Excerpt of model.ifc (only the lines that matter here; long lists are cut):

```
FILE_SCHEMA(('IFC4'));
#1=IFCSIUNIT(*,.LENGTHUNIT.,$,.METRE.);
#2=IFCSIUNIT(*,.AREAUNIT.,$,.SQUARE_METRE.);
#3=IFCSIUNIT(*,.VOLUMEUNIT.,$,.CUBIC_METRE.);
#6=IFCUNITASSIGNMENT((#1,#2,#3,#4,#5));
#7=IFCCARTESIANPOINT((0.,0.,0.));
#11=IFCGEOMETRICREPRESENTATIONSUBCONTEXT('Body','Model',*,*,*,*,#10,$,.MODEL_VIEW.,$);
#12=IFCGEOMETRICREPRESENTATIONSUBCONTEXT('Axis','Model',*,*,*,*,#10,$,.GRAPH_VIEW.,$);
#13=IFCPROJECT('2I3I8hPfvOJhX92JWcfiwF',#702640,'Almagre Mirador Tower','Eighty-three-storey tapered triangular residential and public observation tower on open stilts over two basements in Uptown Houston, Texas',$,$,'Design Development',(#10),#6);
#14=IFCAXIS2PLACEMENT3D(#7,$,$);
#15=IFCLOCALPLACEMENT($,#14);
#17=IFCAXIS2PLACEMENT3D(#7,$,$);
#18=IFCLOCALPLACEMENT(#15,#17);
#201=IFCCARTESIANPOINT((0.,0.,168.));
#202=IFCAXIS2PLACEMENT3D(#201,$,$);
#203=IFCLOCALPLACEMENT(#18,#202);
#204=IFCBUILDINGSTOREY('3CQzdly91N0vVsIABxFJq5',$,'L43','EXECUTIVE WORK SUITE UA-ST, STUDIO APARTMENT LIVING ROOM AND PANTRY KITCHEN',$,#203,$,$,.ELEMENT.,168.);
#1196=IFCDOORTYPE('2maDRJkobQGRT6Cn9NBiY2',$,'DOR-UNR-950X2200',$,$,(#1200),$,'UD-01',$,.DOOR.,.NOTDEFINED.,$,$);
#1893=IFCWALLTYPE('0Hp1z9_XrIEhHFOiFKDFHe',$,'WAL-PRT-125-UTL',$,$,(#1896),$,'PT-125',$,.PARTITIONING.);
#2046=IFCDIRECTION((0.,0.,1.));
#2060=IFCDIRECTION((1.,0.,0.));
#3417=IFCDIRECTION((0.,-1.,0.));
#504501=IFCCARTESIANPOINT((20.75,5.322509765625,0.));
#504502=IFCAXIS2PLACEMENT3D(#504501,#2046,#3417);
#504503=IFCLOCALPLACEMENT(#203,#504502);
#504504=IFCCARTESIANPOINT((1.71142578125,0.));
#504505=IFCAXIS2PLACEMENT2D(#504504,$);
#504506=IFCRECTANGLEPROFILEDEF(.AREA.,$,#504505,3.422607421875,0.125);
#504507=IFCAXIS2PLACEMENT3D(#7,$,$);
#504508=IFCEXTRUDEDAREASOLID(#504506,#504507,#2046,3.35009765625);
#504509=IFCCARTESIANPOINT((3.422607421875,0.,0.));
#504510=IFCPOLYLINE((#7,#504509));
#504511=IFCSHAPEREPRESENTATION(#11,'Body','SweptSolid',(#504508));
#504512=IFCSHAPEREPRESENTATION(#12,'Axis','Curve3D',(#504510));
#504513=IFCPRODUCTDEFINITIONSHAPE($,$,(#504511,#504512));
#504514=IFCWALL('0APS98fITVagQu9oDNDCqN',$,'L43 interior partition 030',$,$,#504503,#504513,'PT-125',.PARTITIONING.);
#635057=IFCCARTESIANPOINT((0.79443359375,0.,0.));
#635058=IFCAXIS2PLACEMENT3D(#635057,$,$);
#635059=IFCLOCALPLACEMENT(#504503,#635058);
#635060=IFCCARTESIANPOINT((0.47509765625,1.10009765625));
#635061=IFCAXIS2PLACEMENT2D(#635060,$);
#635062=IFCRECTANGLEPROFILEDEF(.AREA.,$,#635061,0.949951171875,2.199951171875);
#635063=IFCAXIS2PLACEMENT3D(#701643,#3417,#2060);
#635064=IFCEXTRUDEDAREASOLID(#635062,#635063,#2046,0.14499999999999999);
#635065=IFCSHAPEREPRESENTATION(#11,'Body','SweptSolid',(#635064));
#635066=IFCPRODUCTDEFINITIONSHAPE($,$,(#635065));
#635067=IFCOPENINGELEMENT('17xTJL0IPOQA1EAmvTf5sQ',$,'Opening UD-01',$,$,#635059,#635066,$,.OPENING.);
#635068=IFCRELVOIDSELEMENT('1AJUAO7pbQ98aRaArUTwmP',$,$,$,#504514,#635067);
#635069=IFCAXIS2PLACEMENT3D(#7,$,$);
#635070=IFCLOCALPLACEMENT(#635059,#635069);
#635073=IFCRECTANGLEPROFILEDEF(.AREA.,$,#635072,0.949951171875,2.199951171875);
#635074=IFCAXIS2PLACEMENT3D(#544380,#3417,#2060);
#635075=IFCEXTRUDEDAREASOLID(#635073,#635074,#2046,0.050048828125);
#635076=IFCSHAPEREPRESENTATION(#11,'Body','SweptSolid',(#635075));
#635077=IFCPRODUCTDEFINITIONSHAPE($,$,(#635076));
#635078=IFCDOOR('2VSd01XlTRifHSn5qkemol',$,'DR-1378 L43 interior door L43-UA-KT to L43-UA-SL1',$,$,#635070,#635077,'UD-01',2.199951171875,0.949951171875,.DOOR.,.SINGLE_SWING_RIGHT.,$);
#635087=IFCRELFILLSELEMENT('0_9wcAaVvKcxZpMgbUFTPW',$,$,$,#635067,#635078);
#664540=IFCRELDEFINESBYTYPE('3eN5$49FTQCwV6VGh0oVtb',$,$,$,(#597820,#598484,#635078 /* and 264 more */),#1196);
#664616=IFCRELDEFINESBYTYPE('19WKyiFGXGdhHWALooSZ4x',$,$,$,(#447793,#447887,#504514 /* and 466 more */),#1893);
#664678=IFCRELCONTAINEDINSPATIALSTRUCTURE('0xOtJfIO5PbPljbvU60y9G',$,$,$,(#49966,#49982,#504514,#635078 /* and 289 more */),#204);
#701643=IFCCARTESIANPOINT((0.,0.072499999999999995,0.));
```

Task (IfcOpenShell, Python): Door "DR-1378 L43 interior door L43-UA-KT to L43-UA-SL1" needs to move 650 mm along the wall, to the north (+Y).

```python
import ifcopenshell
import ifcopenshell.api.geometry
import ifcopenshell.util.placement
import ifcopenshell.util.unit

model = ifcopenshell.open("model.ifc")
unit_scale = ifcopenshell.util.unit.calculate_unit_scale(model)

door = model.by_guid("2VSd01XlTRifHSn5qkemol")
opening = door.FillsVoids[0].RelatingOpeningElement
wall = opening.VoidsElements[0].RelatingBuildingElement

wall_matrix = ifcopenshell.util.placement.get_local_placement(wall.ObjectPlacement)
shift = wall_matrix[:3, 0] * -0.65 / unit_scale
before = ifcopenshell.util.placement.get_local_placement(door.ObjectPlacement)[:3, 3].copy()

# The door is placed relative to its opening, so it follows when the opening moves.
matrix = ifcopenshell.util.placement.get_local_placement(opening.ObjectPlacement)
matrix[:3, 3] += shift
ifcopenshell.api.geometry.edit_object_placement(
    model, product=opening, matrix=matrix, is_si=False, should_transform_children=True
)

after = ifcopenshell.util.placement.get_local_placement(door.ObjectPlacement)[:3, 3]
print("door moved by", (after - before).round(3) + 0.0)

model.write("model_v2.ifc")
```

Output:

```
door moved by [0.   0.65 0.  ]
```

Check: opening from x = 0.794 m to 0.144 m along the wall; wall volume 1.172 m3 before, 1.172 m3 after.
